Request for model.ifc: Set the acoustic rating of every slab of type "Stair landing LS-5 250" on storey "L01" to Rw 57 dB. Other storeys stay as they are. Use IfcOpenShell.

First a look at what the model holds.

```python
import ifcopenshell
import ifcopenshell.util.element

model = ifcopenshell.open("model.ifc")
print(model.schema)
storey = next(s for s in model.by_type("IfcBuildingStorey") if s.Name == "L01")
slabs = [e for e in ifcopenshell.util.element.get_decomposition(storey) if e.is_a("IfcSlab")]
seen = {}
for e in slabs:
    element_type = ifcopenshell.util.element.get_type(e)
    key = (element_type.Name if element_type != e and element_type else None, ifcopenshell.util.element.get_pset(e, "Pset_SlabCommon", "AcousticRating"))
    seen[key] = seen.get(key, 0) + 1
for (name, value), count in sorted(seen.items(), key=str):
    print(count, "x", name, "|", value)
```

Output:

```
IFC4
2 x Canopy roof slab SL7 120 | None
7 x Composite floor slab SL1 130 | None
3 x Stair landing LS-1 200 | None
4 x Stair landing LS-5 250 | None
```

```python
import ifcopenshell
import ifcopenshell.api.pset
import ifcopenshell.util.element

model = ifcopenshell.open("model.ifc")

storey = next(s for s in model.by_type("IfcBuildingStorey") if s.Name == "L01")
slabs = [e for e in ifcopenshell.util.element.get_decomposition(storey) if e.is_a("IfcSlab")]

count = 0
for e in slabs:
    element_type = ifcopenshell.util.element.get_type(e)
    if element_type in (None, e) or element_type.Name != "Stair landing LS-5 250":
        continue
    # add_pset returns the element's existing set when there is one.
    pset = ifcopenshell.api.pset.add_pset(model, product=e, name="Pset_SlabCommon")
    ifcopenshell.api.pset.edit_pset(model, pset=pset, properties={"AcousticRating": "Rw 57 dB"})
    count += 1

print(count, "slabs updated")

model.write("model_rev.ifc")
```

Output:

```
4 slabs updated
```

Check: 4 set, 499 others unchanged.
